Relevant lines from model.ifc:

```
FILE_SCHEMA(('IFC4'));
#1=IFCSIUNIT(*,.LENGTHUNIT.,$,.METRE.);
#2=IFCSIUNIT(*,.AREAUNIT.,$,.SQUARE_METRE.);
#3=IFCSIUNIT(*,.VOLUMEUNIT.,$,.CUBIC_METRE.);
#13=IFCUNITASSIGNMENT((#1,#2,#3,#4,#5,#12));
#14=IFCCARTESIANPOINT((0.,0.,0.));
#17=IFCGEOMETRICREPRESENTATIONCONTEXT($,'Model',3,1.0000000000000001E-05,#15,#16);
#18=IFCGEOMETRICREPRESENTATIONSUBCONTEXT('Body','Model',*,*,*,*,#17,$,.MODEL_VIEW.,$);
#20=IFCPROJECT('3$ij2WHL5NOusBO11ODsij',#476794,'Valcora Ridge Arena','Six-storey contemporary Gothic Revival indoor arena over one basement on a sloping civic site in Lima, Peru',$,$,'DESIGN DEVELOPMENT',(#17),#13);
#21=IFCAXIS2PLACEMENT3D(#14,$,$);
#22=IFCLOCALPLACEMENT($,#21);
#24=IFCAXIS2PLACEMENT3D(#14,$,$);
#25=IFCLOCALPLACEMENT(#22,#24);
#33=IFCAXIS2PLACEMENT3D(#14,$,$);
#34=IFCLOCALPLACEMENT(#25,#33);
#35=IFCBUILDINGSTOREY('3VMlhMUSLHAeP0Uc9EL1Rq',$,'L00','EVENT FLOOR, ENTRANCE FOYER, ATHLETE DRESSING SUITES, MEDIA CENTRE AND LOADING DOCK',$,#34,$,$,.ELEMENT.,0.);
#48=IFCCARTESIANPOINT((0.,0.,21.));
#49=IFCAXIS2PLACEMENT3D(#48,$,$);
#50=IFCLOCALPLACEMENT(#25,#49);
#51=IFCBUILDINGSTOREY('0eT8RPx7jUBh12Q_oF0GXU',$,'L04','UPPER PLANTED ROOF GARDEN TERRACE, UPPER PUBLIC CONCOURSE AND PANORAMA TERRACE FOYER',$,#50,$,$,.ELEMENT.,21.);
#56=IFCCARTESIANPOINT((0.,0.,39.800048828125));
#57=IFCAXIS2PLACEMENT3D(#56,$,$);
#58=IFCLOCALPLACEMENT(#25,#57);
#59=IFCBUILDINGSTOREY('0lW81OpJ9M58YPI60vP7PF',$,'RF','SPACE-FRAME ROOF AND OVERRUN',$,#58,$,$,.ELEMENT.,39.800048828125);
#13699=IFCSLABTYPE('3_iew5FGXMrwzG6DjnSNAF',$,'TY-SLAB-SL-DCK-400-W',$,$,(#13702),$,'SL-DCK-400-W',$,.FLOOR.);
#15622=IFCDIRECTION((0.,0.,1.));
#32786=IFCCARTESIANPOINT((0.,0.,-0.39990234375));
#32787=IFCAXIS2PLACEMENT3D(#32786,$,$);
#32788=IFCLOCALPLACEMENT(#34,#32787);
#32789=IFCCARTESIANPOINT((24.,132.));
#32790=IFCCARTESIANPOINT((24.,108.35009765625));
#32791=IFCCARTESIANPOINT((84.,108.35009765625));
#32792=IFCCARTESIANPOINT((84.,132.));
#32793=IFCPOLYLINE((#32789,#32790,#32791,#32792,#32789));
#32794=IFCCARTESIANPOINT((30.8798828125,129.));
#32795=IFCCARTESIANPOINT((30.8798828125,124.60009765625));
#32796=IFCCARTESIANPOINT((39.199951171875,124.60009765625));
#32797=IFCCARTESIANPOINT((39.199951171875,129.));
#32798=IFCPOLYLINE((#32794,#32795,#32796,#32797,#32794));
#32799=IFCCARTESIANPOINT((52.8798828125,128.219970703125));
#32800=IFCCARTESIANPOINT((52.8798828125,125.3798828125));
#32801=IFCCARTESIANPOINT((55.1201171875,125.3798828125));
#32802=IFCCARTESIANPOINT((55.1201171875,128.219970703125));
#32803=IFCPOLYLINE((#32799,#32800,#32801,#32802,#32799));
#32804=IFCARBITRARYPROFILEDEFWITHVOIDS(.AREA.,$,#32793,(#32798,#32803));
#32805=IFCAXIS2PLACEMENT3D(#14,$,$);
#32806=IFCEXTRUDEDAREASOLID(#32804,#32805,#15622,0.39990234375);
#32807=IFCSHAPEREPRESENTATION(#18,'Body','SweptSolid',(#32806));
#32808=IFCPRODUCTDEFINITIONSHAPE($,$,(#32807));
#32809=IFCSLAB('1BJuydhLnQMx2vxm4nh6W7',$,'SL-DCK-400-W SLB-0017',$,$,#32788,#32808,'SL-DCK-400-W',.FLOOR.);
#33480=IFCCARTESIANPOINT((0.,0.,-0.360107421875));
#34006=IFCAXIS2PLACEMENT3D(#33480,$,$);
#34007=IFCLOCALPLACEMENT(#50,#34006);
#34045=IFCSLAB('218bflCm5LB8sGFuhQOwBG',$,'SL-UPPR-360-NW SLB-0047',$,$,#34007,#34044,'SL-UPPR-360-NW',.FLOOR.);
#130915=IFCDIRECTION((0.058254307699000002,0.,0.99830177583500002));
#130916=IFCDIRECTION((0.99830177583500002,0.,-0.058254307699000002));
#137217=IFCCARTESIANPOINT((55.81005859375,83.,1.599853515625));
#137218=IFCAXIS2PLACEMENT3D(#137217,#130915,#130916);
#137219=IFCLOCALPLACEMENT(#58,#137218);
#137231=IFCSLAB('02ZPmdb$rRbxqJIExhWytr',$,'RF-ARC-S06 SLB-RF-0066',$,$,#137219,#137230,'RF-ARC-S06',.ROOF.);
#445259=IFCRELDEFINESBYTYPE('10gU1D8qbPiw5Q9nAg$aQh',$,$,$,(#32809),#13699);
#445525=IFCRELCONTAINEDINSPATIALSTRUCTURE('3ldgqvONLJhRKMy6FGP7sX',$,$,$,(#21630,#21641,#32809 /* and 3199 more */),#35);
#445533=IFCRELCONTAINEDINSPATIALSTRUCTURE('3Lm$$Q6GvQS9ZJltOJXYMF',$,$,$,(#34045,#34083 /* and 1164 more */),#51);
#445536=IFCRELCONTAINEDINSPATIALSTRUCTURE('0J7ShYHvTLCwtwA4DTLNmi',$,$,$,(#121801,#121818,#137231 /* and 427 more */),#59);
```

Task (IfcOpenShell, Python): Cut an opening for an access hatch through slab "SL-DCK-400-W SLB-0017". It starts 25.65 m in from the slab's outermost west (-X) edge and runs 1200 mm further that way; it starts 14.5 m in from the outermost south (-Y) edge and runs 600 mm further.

```python
import numpy as np
import ifcopenshell
import ifcopenshell.api.feature
import ifcopenshell.api.geometry
import ifcopenshell.api.root
import ifcopenshell.geom
import ifcopenshell.util.placement
import ifcopenshell.util.representation
import ifcopenshell.util.shape
import ifcopenshell.util.unit

model = ifcopenshell.open("model.ifc")
unit_scale = ifcopenshell.util.unit.calculate_unit_scale(model)
settings = ifcopenshell.geom.settings()


def volume(element):
    """Net volume in cubic metres, openings subtracted."""
    shape = ifcopenshell.geom.create_shape(settings, element)
    return ifcopenshell.util.shape.get_volume(shape.geometry)


slab = model.by_guid("1BJuydhLnQMx2vxm4nh6W7")
before = volume(slab)

# Extent in the slab's own axes, in metres. The edges named are its -X and -Y sides.
slab_shape = ifcopenshell.geom.create_shape(settings, slab)
vertices = ifcopenshell.util.shape.get_vertices(slab_shape.geometry)
x_min, y_min, bottom = vertices.min(axis=0)
top = vertices[:, 2].max()

opening = ifcopenshell.api.root.create_entity(model, ifc_class="IfcOpeningElement", name="Access hatch opening", predefined_type="OPENING")
context = ifcopenshell.util.representation.get_context(model, "Model", "Body", "MODEL_VIEW")
width, depth = 1.2, 0.6
outline = [(0.0, 0.0), (width, 0.0), (width, depth), (0.0, depth), (0.0, 0.0)]
# Overshoot both faces by 50 mm so the cut is clean.
shape = ifcopenshell.api.geometry.add_slab_representation(
    model, context=context, depth=top - bottom + 0.1, polyline=outline
)
ifcopenshell.api.geometry.assign_representation(model, product=opening, representation=shape)

matrix = ifcopenshell.util.placement.get_local_placement(slab.ObjectPlacement)
matrix[:, 3] = matrix @ np.append(np.array([x_min + 25.65, y_min + 14.5, bottom - 0.05]) / unit_scale, 1.0)
ifcopenshell.api.geometry.edit_object_placement(model, product=opening, matrix=matrix, is_si=False)
ifcopenshell.api.feature.add_feature(model, feature=opening, element=slab)

after = volume(slab)

print(f"slab volume {before:.3f} -> {after:.3f} m3")

model.write("model_v2.ifc")
```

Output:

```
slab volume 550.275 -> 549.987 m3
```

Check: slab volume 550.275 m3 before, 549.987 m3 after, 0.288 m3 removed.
